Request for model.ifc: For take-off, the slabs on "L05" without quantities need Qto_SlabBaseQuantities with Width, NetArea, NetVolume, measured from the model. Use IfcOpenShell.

First a look at what the model holds.

```python
import ifcopenshell
import ifcopenshell.util.element
import ifcopenshell.util.unit

model = ifcopenshell.open("model.ifc")
print(model.schema)
for unit_type in ("LENGTHUNIT", "AREAUNIT", "VOLUMEUNIT"):
    print(unit_type, ifcopenshell.util.unit.calculate_unit_scale(model, unit_type))
storey = next(s for s in model.by_type("IfcBuildingStorey") if s.Name == "L05")
slabs = [e for e in ifcopenshell.util.element.get_decomposition(storey) if e.is_a("IfcSlab")]
for e in sorted(slabs, key=lambda e: e.id()):
    print(e.id(), e.is_a(), e.Name, list(ifcopenshell.util.element.get_psets(e, qtos_only=True)), sep=" | ")
```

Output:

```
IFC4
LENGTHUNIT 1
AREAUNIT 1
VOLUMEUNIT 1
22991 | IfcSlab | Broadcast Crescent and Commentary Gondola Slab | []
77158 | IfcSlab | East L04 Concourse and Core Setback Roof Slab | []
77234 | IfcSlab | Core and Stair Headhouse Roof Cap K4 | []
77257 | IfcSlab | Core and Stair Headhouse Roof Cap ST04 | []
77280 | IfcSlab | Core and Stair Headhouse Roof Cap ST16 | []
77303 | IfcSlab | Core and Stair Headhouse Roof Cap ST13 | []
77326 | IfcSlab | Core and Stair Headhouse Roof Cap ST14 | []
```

```python
import ifcopenshell
import ifcopenshell.api.pset
import ifcopenshell.geom
import ifcopenshell.util.element
import ifcopenshell.util.shape
import ifcopenshell.util.unit

model = ifcopenshell.open("model.ifc")
unit_scale = ifcopenshell.util.unit.calculate_unit_scale(model)
area_scale = ifcopenshell.util.unit.calculate_unit_scale(model, "AREAUNIT")
volume_scale = ifcopenshell.util.unit.calculate_unit_scale(model, "VOLUMEUNIT")
settings = ifcopenshell.geom.settings()

storey = next(s for s in model.by_type("IfcBuildingStorey") if s.Name == "L05")
slabs = [e for e in ifcopenshell.util.element.get_decomposition(storey) if e.is_a("IfcSlab")]

for e in sorted(slabs, key=lambda e: e.id()):
    if ifcopenshell.util.element.get_psets(e, qtos_only=True, should_inherit=False):
        continue
    # Geometry comes back in metres, in the element's own axes.
    shape = ifcopenshell.geom.create_shape(settings, e)
    values = {
        "Width": ifcopenshell.util.shape.get_z(shape.geometry) / unit_scale,
        "NetArea": ifcopenshell.util.shape.get_footprint_area(shape.geometry) / area_scale,
        "NetVolume": ifcopenshell.util.shape.get_volume(shape.geometry) / volume_scale,
    }
    qto = ifcopenshell.api.pset.add_qto(model, product=e, name="Qto_SlabBaseQuantities")
    ifcopenshell.api.pset.edit_qto(model, qto=qto, properties=values)
    print(e.id(), {k: round(v, 3) for k, v in values.items()})

model.write("model_rev.ifc")
```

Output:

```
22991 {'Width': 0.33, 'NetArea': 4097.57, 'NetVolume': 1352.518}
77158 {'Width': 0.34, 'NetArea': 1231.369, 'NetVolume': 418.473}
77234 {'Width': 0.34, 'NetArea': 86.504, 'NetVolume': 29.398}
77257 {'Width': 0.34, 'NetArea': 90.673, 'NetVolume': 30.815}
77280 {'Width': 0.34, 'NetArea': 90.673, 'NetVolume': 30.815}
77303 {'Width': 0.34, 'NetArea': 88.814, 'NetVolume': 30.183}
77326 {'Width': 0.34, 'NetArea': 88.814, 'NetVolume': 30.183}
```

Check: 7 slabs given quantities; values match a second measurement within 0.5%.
